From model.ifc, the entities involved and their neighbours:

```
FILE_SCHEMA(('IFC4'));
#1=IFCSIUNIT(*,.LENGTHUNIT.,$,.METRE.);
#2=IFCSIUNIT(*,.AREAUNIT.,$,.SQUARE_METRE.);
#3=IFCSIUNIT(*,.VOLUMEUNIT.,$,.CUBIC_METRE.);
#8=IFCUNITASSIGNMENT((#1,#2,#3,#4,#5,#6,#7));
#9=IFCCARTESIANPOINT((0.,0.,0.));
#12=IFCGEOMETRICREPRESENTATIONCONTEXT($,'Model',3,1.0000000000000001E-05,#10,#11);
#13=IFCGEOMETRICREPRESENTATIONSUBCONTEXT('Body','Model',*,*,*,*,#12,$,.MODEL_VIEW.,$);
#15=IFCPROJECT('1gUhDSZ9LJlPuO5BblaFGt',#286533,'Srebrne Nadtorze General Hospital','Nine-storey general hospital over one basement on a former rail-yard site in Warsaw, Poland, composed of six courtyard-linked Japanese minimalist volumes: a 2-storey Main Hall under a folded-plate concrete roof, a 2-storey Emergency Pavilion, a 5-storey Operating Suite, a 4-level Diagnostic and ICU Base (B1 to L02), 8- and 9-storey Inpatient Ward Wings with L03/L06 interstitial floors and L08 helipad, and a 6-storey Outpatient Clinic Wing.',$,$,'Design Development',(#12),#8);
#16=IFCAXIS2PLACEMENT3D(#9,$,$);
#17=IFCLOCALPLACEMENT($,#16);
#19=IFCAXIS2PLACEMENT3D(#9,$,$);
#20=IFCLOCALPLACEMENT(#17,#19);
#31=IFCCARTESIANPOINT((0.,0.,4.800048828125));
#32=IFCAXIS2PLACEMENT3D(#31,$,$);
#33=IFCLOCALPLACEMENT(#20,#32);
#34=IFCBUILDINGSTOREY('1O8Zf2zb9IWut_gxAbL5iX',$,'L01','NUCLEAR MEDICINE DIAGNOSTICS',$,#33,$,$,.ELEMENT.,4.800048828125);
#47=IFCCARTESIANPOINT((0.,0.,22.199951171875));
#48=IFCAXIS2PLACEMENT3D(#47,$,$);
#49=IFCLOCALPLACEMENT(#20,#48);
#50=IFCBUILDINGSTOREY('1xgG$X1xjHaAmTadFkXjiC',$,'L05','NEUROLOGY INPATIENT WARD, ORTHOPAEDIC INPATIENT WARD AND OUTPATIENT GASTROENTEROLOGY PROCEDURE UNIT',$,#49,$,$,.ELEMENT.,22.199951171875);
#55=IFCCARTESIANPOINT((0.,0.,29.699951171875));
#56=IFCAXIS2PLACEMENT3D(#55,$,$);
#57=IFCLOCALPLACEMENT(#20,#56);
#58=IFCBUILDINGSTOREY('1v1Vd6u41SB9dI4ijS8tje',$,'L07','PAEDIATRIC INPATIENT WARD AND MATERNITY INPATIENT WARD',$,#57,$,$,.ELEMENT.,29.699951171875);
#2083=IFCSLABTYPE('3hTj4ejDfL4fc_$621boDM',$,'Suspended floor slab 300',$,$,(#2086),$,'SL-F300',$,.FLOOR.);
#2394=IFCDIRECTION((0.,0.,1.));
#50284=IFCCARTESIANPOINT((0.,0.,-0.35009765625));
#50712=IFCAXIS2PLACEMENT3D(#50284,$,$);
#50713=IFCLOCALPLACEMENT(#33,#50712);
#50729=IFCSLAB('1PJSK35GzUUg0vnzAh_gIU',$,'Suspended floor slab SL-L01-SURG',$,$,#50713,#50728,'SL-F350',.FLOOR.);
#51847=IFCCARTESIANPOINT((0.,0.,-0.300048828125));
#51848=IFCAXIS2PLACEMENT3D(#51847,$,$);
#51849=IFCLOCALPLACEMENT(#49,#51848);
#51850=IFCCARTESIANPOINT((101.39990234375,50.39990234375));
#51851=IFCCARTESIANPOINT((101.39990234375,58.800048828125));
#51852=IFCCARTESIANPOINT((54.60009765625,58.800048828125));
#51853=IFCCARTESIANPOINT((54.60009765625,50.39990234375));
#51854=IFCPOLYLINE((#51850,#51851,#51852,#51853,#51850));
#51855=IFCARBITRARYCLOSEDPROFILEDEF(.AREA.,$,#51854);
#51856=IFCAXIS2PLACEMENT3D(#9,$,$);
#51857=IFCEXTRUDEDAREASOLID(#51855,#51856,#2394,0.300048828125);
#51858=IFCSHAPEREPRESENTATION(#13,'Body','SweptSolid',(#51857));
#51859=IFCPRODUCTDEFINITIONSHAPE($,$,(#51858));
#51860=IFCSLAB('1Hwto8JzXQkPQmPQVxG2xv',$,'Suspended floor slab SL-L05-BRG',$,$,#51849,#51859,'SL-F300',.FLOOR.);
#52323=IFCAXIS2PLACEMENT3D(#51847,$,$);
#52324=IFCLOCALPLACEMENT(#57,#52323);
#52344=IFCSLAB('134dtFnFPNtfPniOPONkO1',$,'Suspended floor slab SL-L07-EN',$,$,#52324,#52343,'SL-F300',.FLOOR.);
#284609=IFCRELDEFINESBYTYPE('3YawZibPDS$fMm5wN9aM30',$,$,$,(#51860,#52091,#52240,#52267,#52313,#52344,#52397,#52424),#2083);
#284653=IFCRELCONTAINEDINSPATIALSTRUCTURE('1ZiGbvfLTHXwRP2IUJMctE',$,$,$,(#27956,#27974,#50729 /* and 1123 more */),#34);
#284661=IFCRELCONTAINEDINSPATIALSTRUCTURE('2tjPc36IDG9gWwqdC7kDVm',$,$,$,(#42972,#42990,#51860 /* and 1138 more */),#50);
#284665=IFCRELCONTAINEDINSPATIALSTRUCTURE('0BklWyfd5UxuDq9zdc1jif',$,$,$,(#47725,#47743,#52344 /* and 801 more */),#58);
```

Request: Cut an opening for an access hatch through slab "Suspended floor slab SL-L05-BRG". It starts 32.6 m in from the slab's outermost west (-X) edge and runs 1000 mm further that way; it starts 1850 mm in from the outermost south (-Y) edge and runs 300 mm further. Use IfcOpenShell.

```python
import numpy as np
import ifcopenshell
import ifcopenshell.api.feature
import ifcopenshell.api.geometry
import ifcopenshell.api.root
import ifcopenshell.geom
import ifcopenshell.util.placement
import ifcopenshell.util.representation
import ifcopenshell.util.shape
import ifcopenshell.util.unit

model = ifcopenshell.open("model.ifc")
unit_scale = ifcopenshell.util.unit.calculate_unit_scale(model)
settings = ifcopenshell.geom.settings()


def volume(element):
    """Net volume in cubic metres, openings subtracted."""
    shape = ifcopenshell.geom.create_shape(settings, element)
    return ifcopenshell.util.shape.get_volume(shape.geometry)


slab = model.by_guid("1Hwto8JzXQkPQmPQVxG2xv")
before = volume(slab)

# Extent in the slab's own axes, in metres. The edges named are its -X and -Y sides.
slab_shape = ifcopenshell.geom.create_shape(settings, slab)
vertices = ifcopenshell.util.shape.get_vertices(slab_shape.geometry)
x_min, y_min, bottom = vertices.min(axis=0)
top = vertices[:, 2].max()

opening = ifcopenshell.api.root.create_entity(model, ifc_class="IfcOpeningElement", name="Access hatch opening", predefined_type="OPENING")
context = ifcopenshell.util.representation.get_context(model, "Model", "Body", "MODEL_VIEW")
width, depth = 1, 0.3
outline = [(0.0, 0.0), (width, 0.0), (width, depth), (0.0, depth), (0.0, 0.0)]
# Overshoot both faces by 50 mm so the cut is clean.
shape = ifcopenshell.api.geometry.add_slab_representation(
    model, context=context, depth=top - bottom + 0.1, polyline=outline
)
ifcopenshell.api.geometry.assign_representation(model, product=opening, representation=shape)

matrix = ifcopenshell.util.placement.get_local_placement(slab.ObjectPlacement)
matrix[:, 3] = matrix @ np.append(np.array([x_min + 32.6, y_min + 1.85, bottom - 0.05]) / unit_scale, 1.0)
ifcopenshell.api.geometry.edit_object_placement(model, product=opening, matrix=matrix, is_si=False)
ifcopenshell.api.feature.add_feature(model, feature=opening, element=slab)

after = volume(slab)

print(f"slab volume {before:.3f} -> {after:.3f} m3")

model.write("model_updated.ifc")
```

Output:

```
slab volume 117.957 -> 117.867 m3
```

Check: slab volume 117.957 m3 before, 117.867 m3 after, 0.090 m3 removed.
